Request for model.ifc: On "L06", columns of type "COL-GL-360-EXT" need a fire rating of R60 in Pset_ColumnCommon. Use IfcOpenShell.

First a look at what the model holds.

```python
import ifcopenshell
import ifcopenshell.util.element

model = ifcopenshell.open("model.ifc")
print(model.schema)
storey = next(s for s in model.by_type("IfcBuildingStorey") if s.Name == "L06")
columns = [e for e in ifcopenshell.util.element.get_decomposition(storey) if e.is_a("IfcColumn")]
seen = {}
for e in columns:
    element_type = ifcopenshell.util.element.get_type(e)
    key = (element_type.Name if element_type != e and element_type else None, ifcopenshell.util.element.get_pset(e, "Pset_ColumnCommon", "FireRating"))
    seen[key] = seen.get(key, 0) + 1
for (name, value), count in sorted(seen.items(), key=str):
    print(count, "x", name, "|", value)
```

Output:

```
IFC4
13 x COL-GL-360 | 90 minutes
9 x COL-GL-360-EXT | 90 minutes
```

```python
import ifcopenshell
import ifcopenshell.api.pset
import ifcopenshell.util.element

model = ifcopenshell.open("model.ifc")

storey = next(s for s in model.by_type("IfcBuildingStorey") if s.Name == "L06")
columns = [e for e in ifcopenshell.util.element.get_decomposition(storey) if e.is_a("IfcColumn")]

count = 0
for e in columns:
    element_type = ifcopenshell.util.element.get_type(e)
    if element_type in (None, e) or element_type.Name != "COL-GL-360-EXT":
        continue
    # add_pset returns the element's existing set when there is one.
    pset = ifcopenshell.api.pset.add_pset(model, product=e, name="Pset_ColumnCommon")
    ifcopenshell.api.pset.edit_pset(model, pset=pset, properties={"FireRating": "R60"})
    count += 1

print(count, "columns updated")

model.write("model_rev.ifc")
```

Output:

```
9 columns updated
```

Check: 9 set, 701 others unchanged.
